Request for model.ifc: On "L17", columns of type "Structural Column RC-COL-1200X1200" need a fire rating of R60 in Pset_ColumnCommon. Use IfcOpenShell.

First a look at what the model holds.

```python
import ifcopenshell
import ifcopenshell.util.element

model = ifcopenshell.open("model.ifc")
print(model.schema)
storey = next(s for s in model.by_type("IfcBuildingStorey") if s.Name == "L17")
columns = [e for e in ifcopenshell.util.element.get_decomposition(storey) if e.is_a("IfcColumn")]
seen = {}
for e in columns:
    element_type = ifcopenshell.util.element.get_type(e)
    key = (element_type.Name if element_type != e and element_type else None, ifcopenshell.util.element.get_pset(e, "Pset_ColumnCommon", "FireRating"))
    seen[key] = seen.get(key, 0) + 1
for (name, value), count in sorted(seen.items(), key=str):
    print(count, "x", name, "|", value)
```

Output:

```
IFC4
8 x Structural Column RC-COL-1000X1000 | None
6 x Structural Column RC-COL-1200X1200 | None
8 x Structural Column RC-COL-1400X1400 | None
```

```python
import ifcopenshell
import ifcopenshell.api.pset
import ifcopenshell.util.element

model = ifcopenshell.open("model.ifc")

storey = next(s for s in model.by_type("IfcBuildingStorey") if s.Name == "L17")
columns = [e for e in ifcopenshell.util.element.get_decomposition(storey) if e.is_a("IfcColumn")]

count = 0
for e in columns:
    element_type = ifcopenshell.util.element.get_type(e)
    if element_type in (None, e) or element_type.Name != "Structural Column RC-COL-1200X1200":
        continue
    found = ifcopenshell.util.element.get_pset(e, "Pset_ColumnCommon", should_inherit=False)
    if found:
        pset = model.by_id(found["id"])
        if len(ifcopenshell.util.element.get_elements_by_pset(pset)) > 1:
            pset = ifcopenshell.api.pset.unshare_pset(model, products=[e], pset=pset)[0]
    else:
        pset = ifcopenshell.api.pset.add_pset(model, product=e, name="Pset_ColumnCommon")
    ifcopenshell.api.pset.edit_pset(model, pset=pset, properties={"FireRating": "R60"})
    count += 1

print(count, "columns updated")

model.write("model_v2.ifc")
```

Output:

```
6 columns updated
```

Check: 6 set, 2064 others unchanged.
